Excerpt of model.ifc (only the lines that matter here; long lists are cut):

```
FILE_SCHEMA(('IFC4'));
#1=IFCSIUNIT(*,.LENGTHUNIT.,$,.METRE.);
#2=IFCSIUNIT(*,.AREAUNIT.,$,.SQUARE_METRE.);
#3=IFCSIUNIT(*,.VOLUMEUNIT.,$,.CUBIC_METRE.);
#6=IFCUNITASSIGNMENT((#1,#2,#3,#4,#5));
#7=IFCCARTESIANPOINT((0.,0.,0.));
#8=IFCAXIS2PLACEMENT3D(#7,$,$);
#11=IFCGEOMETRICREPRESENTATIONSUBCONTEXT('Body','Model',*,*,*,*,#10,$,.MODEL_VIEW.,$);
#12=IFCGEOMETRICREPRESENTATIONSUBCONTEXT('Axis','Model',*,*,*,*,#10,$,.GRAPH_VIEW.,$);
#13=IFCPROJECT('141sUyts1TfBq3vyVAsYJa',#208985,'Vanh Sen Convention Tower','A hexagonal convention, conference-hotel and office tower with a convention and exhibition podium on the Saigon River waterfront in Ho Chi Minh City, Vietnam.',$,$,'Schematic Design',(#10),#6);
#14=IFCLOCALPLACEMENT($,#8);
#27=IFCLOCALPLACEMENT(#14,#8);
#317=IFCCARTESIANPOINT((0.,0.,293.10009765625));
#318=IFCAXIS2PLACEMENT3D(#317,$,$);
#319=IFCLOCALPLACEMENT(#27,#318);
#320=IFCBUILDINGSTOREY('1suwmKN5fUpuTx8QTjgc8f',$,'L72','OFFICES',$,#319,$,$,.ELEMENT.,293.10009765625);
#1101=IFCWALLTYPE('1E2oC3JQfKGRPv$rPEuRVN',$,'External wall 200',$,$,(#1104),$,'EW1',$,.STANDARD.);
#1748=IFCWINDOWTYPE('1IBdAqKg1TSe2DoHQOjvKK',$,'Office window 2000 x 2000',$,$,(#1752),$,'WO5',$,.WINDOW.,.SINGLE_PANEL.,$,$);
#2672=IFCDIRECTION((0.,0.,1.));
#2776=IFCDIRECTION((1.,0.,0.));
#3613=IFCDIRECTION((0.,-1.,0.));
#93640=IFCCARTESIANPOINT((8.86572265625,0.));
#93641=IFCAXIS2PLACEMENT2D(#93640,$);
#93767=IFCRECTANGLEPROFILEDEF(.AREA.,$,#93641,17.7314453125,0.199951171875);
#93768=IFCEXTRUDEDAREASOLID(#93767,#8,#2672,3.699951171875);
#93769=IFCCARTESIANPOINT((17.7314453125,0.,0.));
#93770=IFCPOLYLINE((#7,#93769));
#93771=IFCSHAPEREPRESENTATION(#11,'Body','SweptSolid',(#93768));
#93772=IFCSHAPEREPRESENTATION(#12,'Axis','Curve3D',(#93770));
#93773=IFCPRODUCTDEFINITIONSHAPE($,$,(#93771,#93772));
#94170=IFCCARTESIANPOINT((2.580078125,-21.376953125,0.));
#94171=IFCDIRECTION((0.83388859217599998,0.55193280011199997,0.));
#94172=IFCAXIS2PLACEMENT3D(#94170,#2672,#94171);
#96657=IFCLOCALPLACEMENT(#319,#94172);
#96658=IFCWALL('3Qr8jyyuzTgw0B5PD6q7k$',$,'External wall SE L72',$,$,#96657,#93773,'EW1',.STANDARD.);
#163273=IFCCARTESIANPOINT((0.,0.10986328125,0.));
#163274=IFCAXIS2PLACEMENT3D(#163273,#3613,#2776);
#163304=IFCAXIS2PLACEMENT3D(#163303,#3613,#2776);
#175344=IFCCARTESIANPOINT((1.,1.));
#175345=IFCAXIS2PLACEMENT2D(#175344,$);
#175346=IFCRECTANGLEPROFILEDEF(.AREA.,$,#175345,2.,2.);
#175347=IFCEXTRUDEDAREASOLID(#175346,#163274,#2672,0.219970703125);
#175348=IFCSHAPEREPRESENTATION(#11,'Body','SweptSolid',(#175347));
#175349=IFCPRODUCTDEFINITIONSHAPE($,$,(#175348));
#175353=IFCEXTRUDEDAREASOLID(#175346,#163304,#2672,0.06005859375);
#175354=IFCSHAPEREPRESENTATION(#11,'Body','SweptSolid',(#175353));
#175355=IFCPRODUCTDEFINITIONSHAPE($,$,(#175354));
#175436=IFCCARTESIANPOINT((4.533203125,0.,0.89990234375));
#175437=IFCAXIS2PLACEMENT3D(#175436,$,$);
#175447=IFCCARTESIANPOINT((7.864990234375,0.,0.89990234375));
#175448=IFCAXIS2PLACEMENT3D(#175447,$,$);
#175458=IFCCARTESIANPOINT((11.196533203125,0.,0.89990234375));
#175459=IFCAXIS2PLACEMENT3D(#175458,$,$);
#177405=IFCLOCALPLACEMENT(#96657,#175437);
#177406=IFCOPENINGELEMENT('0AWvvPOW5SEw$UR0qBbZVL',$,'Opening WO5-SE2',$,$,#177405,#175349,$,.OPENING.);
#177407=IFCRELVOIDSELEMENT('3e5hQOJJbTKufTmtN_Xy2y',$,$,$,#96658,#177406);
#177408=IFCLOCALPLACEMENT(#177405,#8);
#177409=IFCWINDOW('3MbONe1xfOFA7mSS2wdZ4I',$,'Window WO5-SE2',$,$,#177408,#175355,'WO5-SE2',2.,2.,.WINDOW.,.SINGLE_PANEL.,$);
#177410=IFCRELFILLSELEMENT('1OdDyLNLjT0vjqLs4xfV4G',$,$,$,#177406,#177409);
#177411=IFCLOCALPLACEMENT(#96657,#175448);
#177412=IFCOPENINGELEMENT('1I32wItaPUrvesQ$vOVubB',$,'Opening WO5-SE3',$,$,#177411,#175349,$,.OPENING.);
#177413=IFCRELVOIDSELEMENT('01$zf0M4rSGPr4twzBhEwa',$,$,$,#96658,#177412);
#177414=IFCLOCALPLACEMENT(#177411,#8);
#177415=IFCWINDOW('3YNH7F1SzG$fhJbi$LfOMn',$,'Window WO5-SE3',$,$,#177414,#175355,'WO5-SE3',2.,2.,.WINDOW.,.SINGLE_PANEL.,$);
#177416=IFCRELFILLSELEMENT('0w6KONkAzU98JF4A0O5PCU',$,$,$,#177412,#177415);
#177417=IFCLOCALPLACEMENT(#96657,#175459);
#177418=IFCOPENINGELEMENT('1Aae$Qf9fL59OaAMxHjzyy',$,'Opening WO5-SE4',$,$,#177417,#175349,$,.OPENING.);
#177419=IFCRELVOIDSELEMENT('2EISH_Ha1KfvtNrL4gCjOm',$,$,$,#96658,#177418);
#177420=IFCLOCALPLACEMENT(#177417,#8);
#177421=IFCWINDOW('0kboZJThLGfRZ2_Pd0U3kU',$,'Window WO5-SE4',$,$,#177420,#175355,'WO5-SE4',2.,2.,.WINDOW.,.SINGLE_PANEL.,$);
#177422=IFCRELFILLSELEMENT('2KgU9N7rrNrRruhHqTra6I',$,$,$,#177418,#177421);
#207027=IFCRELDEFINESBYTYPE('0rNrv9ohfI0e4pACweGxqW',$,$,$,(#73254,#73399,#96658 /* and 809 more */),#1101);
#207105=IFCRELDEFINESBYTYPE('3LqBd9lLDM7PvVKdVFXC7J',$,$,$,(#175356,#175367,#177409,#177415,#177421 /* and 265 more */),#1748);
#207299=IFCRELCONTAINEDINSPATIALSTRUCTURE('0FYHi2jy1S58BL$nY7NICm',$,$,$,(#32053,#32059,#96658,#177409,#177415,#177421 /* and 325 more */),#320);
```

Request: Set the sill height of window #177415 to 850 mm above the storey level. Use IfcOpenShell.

```python
import numpy as np
import ifcopenshell
import ifcopenshell.api.geometry
import ifcopenshell.geom
import ifcopenshell.util.element
import ifcopenshell.util.placement
import ifcopenshell.util.shape
import ifcopenshell.util.unit

model = ifcopenshell.open("model.ifc")
unit_scale = ifcopenshell.util.unit.calculate_unit_scale(model)

window = model.by_id(177415)
opening = window.FillsVoids[0].RelatingOpeningElement
storey = ifcopenshell.util.element.get_container(window, ifc_class="IfcBuildingStorey")
level = ifcopenshell.util.placement.get_local_placement(storey.ObjectPlacement)[2, 3]

# The opening's origin need not be at the sill, so measure its lowest point.
shape = ifcopenshell.geom.create_shape(ifcopenshell.geom.settings(), opening)
bottom = ifcopenshell.util.shape.get_shape_bottom_elevation(shape, shape.geometry) / unit_scale
dz = level + 0.85 / unit_scale - bottom

shift = np.array([0.0, 0.0, dz])
# The window is placed relative to its opening, so it follows when the opening moves.
matrix = ifcopenshell.util.placement.get_local_placement(opening.ObjectPlacement)
matrix[:3, 3] += shift
ifcopenshell.api.geometry.edit_object_placement(
    model, product=opening, matrix=matrix, is_si=False, should_transform_children=True
)

print(f"moved by {dz * unit_scale:+.3f} m")

model.write("model_v2.ifc")
```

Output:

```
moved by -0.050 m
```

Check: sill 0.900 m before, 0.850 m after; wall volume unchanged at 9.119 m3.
